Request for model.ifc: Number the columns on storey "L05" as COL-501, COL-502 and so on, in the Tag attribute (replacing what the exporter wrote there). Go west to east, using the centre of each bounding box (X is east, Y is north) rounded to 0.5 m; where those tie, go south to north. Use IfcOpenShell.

First a look at what the model holds.

```python
import ifcopenshell
import ifcopenshell.util.element
import ifcopenshell.util.placement

model = ifcopenshell.open("model.ifc")
print(model.schema)
storey = next(s for s in model.by_type("IfcBuildingStorey") if s.Name == "L05")
columns = [e for e in ifcopenshell.util.element.get_decomposition(storey) if e.is_a("IfcColumn")]
for e in sorted(columns, key=lambda e: e.id()):
    origin = ifcopenshell.util.placement.get_local_placement(e.ObjectPlacement)[:3, 3]
    print(e.id(), e.Tag, e.Name, origin.round(2) + 0.0, sep=" | ")
```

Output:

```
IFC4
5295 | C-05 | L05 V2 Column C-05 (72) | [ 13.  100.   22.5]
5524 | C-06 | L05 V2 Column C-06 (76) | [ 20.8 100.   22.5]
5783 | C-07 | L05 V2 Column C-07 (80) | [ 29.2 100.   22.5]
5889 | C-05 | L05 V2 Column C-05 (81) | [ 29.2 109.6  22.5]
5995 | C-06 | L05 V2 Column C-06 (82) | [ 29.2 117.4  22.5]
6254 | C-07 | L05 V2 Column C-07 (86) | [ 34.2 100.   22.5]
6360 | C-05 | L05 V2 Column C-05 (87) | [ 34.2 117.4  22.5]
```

```python
import ifcopenshell
import ifcopenshell.geom
import ifcopenshell.util.element
import ifcopenshell.util.shape

model = ifcopenshell.open("model.ifc")
settings = ifcopenshell.geom.settings()
settings.set("use-world-coords", True)


def centre(element):
    shape = ifcopenshell.geom.create_shape(settings, element)
    return ifcopenshell.util.shape.get_bbox_centroid(shape.geometry)


storey = next(s for s in model.by_type("IfcBuildingStorey") if s.Name == "L05")
columns = [e for e in ifcopenshell.util.element.get_decomposition(storey) if e.is_a("IfcColumn")]

# Insertion points can sit at a corner or the storey origin, so sort by the geometry (in metres).
centres = {e: centre(e) for e in columns}
columns.sort(key=lambda e: (round(centres[e][0] / 0.5), centres[e][1]))

for i, e in enumerate(columns, start=1):
    number = f"COL-5{i:02d}"
    e.Tag = number
    print(e.id(), number)

model.write("model_rev.ifc")
```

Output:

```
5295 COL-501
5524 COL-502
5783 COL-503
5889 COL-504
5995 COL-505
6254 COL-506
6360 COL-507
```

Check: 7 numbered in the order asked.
